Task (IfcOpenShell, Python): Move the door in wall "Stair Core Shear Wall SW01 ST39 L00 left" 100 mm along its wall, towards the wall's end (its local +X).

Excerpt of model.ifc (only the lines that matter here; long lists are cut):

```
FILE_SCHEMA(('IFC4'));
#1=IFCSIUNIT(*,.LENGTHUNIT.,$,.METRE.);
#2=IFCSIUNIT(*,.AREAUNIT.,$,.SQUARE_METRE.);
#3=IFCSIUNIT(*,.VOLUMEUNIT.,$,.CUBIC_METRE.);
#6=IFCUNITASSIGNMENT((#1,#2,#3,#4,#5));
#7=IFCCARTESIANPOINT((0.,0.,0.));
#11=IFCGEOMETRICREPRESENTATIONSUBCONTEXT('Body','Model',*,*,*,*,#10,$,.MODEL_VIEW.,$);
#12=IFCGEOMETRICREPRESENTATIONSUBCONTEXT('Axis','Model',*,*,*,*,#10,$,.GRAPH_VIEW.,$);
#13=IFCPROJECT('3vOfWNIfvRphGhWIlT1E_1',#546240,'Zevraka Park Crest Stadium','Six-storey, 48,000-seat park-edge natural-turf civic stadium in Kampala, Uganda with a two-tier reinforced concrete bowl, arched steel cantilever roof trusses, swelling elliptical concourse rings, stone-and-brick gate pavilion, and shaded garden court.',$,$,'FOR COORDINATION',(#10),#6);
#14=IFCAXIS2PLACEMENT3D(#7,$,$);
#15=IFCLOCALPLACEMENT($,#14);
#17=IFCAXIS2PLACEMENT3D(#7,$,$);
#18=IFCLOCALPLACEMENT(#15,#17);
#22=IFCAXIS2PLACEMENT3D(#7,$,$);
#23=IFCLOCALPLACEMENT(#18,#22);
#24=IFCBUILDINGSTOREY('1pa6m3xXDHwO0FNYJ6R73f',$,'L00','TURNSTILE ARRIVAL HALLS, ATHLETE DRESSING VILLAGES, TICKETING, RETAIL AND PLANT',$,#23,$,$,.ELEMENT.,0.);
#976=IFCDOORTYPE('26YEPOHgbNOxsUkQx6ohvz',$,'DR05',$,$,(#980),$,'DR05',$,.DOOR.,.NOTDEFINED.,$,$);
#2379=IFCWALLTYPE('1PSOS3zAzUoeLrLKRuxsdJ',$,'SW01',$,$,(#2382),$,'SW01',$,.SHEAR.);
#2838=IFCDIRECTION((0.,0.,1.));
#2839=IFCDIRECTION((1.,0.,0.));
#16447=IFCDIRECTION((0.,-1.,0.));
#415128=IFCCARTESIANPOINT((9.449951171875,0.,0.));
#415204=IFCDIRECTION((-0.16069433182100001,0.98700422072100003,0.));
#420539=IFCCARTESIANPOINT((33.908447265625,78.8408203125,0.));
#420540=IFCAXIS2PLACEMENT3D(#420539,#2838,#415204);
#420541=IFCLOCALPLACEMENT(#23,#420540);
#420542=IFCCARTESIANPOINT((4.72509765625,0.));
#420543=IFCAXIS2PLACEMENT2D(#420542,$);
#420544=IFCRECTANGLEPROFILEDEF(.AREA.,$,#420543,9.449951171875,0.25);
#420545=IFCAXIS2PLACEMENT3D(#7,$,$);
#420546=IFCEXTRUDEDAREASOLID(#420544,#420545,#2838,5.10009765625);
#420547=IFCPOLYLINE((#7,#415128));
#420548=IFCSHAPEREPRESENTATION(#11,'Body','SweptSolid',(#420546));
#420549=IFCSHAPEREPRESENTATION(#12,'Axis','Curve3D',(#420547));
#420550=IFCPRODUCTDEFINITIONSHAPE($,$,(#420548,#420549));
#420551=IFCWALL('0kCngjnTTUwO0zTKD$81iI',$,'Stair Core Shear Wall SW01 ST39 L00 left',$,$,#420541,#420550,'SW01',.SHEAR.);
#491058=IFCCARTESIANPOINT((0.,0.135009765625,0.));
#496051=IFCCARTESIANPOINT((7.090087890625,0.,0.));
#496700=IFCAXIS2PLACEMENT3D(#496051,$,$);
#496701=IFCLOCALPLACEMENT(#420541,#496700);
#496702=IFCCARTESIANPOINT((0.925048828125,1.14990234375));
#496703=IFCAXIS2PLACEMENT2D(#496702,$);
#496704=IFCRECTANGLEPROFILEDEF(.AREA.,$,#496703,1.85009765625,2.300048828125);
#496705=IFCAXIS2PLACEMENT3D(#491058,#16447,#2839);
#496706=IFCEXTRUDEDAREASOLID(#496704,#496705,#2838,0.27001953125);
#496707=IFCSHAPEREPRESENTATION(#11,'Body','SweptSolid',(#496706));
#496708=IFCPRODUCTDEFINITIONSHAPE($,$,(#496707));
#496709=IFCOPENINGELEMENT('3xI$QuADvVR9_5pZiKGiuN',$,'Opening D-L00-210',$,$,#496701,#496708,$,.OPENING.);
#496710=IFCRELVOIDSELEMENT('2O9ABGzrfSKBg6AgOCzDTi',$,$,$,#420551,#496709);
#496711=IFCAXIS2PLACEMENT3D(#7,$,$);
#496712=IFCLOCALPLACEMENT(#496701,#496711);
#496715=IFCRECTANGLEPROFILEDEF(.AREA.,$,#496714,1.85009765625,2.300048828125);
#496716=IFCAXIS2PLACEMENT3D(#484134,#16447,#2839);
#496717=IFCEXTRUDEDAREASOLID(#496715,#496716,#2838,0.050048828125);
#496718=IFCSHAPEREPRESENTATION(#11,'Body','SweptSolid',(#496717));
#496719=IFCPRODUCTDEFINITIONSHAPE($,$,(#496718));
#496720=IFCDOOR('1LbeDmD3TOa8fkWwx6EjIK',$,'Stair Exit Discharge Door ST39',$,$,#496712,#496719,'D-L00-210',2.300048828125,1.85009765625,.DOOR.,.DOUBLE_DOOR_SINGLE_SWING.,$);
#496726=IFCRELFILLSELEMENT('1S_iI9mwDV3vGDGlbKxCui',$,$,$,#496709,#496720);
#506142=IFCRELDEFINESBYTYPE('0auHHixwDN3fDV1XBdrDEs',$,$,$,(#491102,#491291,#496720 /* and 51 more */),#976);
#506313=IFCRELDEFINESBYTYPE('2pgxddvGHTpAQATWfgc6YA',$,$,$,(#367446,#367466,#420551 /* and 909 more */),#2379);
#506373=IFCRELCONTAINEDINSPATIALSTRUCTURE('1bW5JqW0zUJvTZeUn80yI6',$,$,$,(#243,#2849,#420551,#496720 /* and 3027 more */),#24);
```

```python
import ifcopenshell
import ifcopenshell.api.geometry
import ifcopenshell.util.placement
import ifcopenshell.util.unit

model = ifcopenshell.open("model.ifc")
unit_scale = ifcopenshell.util.unit.calculate_unit_scale(model)

door = model.by_id(496720)
opening = door.FillsVoids[0].RelatingOpeningElement
wall = opening.VoidsElements[0].RelatingBuildingElement

wall_matrix = ifcopenshell.util.placement.get_local_placement(wall.ObjectPlacement)
shift = wall_matrix[:3, 0] * 0.1 / unit_scale
before = ifcopenshell.util.placement.get_local_placement(door.ObjectPlacement)[:3, 3].copy()

# The door is placed relative to its opening, so it follows when the opening moves.
matrix = ifcopenshell.util.placement.get_local_placement(opening.ObjectPlacement)
matrix[:3, 3] += shift
ifcopenshell.api.geometry.edit_object_placement(
    model, product=opening, matrix=matrix, is_si=False, should_transform_children=True
)

after = ifcopenshell.util.placement.get_local_placement(door.ObjectPlacement)[:3, 3]
print("door moved by", (after - before).round(3) + 0.0)

model.write("model_updated.ifc")
```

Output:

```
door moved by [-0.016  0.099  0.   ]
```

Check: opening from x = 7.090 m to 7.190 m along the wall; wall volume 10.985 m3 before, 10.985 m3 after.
